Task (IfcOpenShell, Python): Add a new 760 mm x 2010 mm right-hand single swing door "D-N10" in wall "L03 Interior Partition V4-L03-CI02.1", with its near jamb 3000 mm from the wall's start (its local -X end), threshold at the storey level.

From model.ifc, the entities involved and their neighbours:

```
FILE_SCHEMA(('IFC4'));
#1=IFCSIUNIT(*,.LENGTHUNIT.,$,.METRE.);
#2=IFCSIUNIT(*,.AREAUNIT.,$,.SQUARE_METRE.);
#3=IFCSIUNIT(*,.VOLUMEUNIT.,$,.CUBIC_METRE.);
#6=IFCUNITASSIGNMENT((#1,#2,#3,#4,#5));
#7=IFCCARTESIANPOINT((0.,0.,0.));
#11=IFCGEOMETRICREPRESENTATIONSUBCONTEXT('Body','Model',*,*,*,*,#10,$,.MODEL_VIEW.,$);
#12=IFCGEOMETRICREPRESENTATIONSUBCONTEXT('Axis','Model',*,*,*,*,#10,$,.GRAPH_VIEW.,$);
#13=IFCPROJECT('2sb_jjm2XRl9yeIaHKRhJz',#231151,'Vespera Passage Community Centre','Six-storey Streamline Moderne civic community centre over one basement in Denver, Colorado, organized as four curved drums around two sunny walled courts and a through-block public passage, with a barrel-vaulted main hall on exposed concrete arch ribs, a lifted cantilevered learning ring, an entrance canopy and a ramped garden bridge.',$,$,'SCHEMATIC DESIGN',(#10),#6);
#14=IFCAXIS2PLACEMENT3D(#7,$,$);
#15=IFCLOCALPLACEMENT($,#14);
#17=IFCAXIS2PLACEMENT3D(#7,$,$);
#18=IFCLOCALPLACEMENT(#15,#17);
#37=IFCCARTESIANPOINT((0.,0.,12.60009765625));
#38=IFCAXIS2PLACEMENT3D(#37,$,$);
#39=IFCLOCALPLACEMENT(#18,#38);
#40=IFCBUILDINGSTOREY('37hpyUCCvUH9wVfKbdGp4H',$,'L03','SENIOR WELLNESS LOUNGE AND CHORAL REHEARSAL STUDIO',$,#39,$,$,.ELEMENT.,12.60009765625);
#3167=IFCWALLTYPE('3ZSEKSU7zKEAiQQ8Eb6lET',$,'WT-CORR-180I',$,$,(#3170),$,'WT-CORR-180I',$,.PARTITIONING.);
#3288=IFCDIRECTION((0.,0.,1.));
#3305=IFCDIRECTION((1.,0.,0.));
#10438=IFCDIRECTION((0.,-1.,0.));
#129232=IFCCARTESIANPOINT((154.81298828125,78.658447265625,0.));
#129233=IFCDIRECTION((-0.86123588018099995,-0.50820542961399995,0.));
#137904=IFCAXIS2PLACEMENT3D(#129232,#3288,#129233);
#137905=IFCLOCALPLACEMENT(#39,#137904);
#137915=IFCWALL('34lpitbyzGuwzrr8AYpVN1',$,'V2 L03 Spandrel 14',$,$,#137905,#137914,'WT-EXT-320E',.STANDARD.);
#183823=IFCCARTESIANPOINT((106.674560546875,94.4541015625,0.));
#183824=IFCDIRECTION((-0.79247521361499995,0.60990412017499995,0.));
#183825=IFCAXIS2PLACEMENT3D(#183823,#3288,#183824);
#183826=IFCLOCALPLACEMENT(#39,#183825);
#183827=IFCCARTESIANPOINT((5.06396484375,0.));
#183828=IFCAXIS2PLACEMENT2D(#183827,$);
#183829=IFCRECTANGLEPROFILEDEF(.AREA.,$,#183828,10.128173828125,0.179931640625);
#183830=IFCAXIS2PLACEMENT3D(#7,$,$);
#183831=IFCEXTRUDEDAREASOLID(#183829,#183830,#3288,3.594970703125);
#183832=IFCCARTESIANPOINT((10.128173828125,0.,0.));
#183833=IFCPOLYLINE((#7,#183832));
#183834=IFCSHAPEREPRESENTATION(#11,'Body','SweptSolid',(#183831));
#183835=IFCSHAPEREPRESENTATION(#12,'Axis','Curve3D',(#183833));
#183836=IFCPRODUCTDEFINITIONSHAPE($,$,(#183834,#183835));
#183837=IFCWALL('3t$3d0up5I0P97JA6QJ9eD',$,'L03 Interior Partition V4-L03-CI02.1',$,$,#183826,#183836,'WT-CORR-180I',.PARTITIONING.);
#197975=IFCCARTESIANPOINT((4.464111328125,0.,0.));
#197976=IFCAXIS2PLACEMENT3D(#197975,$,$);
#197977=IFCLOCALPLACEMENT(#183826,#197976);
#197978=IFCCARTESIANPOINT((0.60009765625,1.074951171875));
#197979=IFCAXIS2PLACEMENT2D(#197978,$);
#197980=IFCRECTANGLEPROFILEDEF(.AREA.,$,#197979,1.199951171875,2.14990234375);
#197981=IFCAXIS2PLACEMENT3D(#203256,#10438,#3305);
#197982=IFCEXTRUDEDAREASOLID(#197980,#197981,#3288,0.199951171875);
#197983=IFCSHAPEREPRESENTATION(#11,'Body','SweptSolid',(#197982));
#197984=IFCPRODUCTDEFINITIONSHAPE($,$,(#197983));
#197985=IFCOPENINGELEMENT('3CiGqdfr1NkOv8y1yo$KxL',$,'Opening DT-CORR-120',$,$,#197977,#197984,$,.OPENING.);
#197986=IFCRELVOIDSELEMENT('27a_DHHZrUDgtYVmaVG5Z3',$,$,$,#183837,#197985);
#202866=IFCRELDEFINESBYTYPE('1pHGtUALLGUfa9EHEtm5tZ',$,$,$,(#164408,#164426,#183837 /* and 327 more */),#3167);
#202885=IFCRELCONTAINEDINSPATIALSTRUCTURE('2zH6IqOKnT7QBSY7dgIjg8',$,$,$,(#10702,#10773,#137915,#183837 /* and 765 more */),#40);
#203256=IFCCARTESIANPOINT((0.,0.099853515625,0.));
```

```python
import numpy as np
import ifcopenshell
import ifcopenshell.api.feature
import ifcopenshell.api.geometry
import ifcopenshell.api.root
import ifcopenshell.api.spatial
import ifcopenshell.geom
import ifcopenshell.util.element
import ifcopenshell.util.placement
import ifcopenshell.util.representation
import ifcopenshell.util.shape
import ifcopenshell.util.unit

model = ifcopenshell.open("model.ifc")
unit_scale = ifcopenshell.util.unit.calculate_unit_scale(model)
settings = ifcopenshell.geom.settings()


def volume(element):
    """Net volume in cubic metres, openings subtracted."""
    shape = ifcopenshell.geom.create_shape(settings, element)
    return ifcopenshell.util.shape.get_volume(shape.geometry)


wall = model.by_guid("3t$3d0up5I0P97JA6QJ9eD")
storey = ifcopenshell.util.element.get_container(wall, ifc_class="IfcBuildingStorey")
context = ifcopenshell.util.representation.get_context(model, "Model", "Body", "MODEL_VIEW")
before = volume(wall)

width, height, from_end, sill = 0.76, 2.01, 3, 0.0  # metres

# The wall runs along its own X axis, and the end named is its -X end.
wall_shape = ifcopenshell.geom.create_shape(settings, wall)
x, y, z = ifcopenshell.util.shape.get_vertices(wall_shape.geometry).T
start = x.min() + from_end
face, thickness = float(y.min()), float(y.max() - y.min())
wall_matrix = ifcopenshell.util.placement.get_local_placement(wall.ObjectPlacement)
level = ifcopenshell.util.placement.get_local_placement(storey.ObjectPlacement)[2, 3]


def in_wall(x, y):
    """Placement at x, y metres in the wall's axes, at sill height."""
    matrix = wall_matrix.copy()
    matrix[:, 3] = wall_matrix @ np.array([x / unit_scale, y / unit_scale, 0.0, 1.0])
    matrix[2, 3] = level + sill / unit_scale
    return matrix


# Opening: a box that overshoots both wall faces by 50 mm.
opening = ifcopenshell.api.root.create_entity(model, ifc_class="IfcOpeningElement", predefined_type="OPENING")
box = ifcopenshell.api.geometry.add_wall_representation(
    model, context=context, length=width, height=height, thickness=thickness + 0.1
)
ifcopenshell.api.geometry.assign_representation(model, product=opening, representation=box)
ifcopenshell.api.geometry.edit_object_placement(model, product=opening, matrix=in_wall(start, face - 0.05), is_si=False)
ifcopenshell.api.feature.add_feature(model, feature=opening, element=wall)

door = ifcopenshell.api.root.create_entity(model, ifc_class="IfcDoor", name="D-N10", predefined_type="DOOR")
door.OverallWidth, door.OverallHeight = width / unit_scale, height / unit_scale
door.OperationType = "SINGLE_SWING_RIGHT"
body = ifcopenshell.api.geometry.add_door_representation(
    model,
    context=context,
    overall_width=door.OverallWidth,
    overall_height=door.OverallHeight,
    operation_type="SINGLE_SWING_RIGHT",
    lining_properties={"LiningDepth": thickness / unit_scale, "ThresholdDepth": thickness / unit_scale},
)
ifcopenshell.api.geometry.assign_representation(model, product=door, representation=body)
ifcopenshell.api.spatial.assign_container(model, products=[door], relating_structure=storey)
ifcopenshell.api.feature.add_filling(model, opening=opening, element=door)

# The lining spans the wall, so the door starts at the wall face.
ifcopenshell.api.geometry.edit_object_placement(model, product=door, matrix=in_wall(start, face), is_si=False)

after = volume(wall)

print(f"wall volume {before:.3f} -> {after:.3f} m3")

model.write("model_v2.ifc")
```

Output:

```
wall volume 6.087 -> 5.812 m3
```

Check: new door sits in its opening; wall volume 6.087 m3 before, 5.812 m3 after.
